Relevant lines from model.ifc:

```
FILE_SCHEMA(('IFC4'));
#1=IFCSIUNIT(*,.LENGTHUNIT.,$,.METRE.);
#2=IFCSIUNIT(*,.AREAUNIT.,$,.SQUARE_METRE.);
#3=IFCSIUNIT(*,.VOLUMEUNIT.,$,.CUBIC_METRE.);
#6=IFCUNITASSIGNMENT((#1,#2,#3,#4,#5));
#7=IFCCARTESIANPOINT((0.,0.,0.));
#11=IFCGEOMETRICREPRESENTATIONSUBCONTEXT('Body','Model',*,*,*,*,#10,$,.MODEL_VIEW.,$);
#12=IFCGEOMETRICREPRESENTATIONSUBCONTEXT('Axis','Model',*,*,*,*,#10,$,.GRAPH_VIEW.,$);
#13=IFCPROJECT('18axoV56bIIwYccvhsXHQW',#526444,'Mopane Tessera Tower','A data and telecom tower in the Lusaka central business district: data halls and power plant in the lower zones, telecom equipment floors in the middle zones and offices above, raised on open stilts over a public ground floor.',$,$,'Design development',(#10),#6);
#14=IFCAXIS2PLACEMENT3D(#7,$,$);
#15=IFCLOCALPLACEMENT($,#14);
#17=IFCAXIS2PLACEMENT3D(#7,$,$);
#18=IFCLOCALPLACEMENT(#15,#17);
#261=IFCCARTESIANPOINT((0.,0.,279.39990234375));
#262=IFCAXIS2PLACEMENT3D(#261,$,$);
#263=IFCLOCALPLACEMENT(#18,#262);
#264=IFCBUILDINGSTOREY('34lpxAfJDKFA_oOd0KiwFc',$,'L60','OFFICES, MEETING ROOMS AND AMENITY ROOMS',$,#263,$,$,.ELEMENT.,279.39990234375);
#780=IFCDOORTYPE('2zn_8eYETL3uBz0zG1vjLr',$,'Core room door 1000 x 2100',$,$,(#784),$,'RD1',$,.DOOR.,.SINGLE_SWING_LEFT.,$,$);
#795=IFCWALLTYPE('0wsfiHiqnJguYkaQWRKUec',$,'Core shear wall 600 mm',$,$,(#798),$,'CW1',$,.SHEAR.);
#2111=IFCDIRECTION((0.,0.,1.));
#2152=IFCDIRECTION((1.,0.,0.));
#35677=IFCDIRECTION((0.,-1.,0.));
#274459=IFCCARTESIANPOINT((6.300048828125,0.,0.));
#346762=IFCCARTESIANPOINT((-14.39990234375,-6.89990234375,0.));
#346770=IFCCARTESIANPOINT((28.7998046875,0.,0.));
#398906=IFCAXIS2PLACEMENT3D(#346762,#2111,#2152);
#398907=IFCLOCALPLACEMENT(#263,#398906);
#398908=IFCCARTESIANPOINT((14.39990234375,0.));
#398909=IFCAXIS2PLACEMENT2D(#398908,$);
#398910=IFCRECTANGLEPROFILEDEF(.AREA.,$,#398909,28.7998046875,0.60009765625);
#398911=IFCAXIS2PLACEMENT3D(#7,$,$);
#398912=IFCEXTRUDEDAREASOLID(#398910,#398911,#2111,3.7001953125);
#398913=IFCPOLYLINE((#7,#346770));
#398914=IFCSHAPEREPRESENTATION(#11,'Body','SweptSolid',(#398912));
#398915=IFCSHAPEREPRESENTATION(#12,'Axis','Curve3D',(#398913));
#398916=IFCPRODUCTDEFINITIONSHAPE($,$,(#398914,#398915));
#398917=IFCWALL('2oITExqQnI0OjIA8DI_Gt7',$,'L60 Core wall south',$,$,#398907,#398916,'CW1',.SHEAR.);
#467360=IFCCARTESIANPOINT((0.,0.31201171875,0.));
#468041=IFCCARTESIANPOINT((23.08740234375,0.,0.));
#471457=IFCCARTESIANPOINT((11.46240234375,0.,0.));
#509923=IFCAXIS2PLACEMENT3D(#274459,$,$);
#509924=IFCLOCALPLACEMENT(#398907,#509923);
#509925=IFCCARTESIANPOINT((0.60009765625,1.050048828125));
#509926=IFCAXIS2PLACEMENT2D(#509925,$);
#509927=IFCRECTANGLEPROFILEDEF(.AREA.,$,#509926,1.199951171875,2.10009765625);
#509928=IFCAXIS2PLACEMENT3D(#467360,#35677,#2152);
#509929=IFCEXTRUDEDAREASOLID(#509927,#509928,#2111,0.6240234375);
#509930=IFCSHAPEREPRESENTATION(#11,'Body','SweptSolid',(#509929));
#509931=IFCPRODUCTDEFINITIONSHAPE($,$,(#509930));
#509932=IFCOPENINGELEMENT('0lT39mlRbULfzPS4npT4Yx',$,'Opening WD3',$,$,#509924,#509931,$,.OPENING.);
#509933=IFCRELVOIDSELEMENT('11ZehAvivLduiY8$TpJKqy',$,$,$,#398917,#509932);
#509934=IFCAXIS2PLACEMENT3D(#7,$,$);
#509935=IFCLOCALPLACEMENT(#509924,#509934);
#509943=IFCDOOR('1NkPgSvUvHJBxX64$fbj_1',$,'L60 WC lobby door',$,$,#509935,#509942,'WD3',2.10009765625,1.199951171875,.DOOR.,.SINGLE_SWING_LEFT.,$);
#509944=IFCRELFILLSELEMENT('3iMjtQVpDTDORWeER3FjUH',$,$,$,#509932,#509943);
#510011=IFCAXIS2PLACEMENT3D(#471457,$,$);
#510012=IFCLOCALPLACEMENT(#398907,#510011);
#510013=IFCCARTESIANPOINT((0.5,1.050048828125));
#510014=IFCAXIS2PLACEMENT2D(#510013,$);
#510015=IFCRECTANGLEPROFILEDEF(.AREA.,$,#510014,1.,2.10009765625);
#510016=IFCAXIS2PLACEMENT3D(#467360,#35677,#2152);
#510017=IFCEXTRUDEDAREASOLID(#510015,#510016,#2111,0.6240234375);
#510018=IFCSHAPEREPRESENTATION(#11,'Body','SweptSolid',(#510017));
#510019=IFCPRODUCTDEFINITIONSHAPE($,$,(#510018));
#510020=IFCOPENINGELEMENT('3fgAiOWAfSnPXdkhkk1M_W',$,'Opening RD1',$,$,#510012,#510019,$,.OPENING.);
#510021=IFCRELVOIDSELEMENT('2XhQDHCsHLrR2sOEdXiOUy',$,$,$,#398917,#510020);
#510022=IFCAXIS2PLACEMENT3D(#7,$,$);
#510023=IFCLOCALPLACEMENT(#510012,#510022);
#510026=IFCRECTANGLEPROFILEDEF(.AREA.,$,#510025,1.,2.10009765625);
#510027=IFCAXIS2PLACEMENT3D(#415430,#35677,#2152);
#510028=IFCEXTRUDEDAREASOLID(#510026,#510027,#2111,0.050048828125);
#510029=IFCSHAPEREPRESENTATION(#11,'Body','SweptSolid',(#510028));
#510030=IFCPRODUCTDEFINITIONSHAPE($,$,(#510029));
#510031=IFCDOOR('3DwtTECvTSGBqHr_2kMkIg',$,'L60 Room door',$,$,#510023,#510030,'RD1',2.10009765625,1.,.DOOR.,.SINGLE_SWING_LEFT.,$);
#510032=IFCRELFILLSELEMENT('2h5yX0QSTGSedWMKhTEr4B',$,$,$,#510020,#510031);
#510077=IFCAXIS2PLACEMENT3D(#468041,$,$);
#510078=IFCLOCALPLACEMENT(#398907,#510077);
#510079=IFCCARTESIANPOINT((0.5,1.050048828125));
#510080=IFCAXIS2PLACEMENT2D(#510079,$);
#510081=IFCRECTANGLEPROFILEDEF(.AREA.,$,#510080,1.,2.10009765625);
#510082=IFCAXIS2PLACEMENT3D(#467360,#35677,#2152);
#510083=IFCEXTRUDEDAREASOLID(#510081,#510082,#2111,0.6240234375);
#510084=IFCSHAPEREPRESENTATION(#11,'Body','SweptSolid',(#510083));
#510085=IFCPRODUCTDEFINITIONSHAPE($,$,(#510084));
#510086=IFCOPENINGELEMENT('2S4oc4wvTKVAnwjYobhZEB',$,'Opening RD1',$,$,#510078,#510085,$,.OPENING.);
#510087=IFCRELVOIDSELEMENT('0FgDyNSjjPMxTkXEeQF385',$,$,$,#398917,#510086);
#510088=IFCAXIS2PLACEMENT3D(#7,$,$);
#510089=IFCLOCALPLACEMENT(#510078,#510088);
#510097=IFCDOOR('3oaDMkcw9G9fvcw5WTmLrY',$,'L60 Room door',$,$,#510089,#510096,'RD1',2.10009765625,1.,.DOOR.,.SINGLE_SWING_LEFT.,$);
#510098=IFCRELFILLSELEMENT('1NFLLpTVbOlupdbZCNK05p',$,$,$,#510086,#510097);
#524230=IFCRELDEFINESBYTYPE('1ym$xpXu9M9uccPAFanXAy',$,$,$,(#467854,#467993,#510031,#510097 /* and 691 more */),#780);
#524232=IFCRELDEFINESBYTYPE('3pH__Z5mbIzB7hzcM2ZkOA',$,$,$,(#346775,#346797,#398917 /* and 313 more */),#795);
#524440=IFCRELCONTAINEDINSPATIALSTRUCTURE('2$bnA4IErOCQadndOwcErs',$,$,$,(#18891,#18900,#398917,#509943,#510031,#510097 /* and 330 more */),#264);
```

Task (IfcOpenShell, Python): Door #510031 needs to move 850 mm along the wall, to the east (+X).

```python
import ifcopenshell
import ifcopenshell.api.geometry
import ifcopenshell.util.placement
import ifcopenshell.util.unit

model = ifcopenshell.open("model.ifc")
unit_scale = ifcopenshell.util.unit.calculate_unit_scale(model)

door = model.by_guid("3DwtTECvTSGBqHr_2kMkIg")
opening = door.FillsVoids[0].RelatingOpeningElement
wall = opening.VoidsElements[0].RelatingBuildingElement

wall_matrix = ifcopenshell.util.placement.get_local_placement(wall.ObjectPlacement)
shift = wall_matrix[:3, 0] * 0.85 / unit_scale
before = ifcopenshell.util.placement.get_local_placement(door.ObjectPlacement)[:3, 3].copy()

# The door is placed relative to its opening, so it follows when the opening moves.
matrix = ifcopenshell.util.placement.get_local_placement(opening.ObjectPlacement)
matrix[:3, 3] += shift
ifcopenshell.api.geometry.edit_object_placement(
    model, product=opening, matrix=matrix, is_si=False, should_transform_children=True
)

after = ifcopenshell.util.placement.get_local_placement(door.ObjectPlacement)[:3, 3]
print("door moved by", (after - before).round(3) + 0.0)

model.write("model_updated.ifc")
```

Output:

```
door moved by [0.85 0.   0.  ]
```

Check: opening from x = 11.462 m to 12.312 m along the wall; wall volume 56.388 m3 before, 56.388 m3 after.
